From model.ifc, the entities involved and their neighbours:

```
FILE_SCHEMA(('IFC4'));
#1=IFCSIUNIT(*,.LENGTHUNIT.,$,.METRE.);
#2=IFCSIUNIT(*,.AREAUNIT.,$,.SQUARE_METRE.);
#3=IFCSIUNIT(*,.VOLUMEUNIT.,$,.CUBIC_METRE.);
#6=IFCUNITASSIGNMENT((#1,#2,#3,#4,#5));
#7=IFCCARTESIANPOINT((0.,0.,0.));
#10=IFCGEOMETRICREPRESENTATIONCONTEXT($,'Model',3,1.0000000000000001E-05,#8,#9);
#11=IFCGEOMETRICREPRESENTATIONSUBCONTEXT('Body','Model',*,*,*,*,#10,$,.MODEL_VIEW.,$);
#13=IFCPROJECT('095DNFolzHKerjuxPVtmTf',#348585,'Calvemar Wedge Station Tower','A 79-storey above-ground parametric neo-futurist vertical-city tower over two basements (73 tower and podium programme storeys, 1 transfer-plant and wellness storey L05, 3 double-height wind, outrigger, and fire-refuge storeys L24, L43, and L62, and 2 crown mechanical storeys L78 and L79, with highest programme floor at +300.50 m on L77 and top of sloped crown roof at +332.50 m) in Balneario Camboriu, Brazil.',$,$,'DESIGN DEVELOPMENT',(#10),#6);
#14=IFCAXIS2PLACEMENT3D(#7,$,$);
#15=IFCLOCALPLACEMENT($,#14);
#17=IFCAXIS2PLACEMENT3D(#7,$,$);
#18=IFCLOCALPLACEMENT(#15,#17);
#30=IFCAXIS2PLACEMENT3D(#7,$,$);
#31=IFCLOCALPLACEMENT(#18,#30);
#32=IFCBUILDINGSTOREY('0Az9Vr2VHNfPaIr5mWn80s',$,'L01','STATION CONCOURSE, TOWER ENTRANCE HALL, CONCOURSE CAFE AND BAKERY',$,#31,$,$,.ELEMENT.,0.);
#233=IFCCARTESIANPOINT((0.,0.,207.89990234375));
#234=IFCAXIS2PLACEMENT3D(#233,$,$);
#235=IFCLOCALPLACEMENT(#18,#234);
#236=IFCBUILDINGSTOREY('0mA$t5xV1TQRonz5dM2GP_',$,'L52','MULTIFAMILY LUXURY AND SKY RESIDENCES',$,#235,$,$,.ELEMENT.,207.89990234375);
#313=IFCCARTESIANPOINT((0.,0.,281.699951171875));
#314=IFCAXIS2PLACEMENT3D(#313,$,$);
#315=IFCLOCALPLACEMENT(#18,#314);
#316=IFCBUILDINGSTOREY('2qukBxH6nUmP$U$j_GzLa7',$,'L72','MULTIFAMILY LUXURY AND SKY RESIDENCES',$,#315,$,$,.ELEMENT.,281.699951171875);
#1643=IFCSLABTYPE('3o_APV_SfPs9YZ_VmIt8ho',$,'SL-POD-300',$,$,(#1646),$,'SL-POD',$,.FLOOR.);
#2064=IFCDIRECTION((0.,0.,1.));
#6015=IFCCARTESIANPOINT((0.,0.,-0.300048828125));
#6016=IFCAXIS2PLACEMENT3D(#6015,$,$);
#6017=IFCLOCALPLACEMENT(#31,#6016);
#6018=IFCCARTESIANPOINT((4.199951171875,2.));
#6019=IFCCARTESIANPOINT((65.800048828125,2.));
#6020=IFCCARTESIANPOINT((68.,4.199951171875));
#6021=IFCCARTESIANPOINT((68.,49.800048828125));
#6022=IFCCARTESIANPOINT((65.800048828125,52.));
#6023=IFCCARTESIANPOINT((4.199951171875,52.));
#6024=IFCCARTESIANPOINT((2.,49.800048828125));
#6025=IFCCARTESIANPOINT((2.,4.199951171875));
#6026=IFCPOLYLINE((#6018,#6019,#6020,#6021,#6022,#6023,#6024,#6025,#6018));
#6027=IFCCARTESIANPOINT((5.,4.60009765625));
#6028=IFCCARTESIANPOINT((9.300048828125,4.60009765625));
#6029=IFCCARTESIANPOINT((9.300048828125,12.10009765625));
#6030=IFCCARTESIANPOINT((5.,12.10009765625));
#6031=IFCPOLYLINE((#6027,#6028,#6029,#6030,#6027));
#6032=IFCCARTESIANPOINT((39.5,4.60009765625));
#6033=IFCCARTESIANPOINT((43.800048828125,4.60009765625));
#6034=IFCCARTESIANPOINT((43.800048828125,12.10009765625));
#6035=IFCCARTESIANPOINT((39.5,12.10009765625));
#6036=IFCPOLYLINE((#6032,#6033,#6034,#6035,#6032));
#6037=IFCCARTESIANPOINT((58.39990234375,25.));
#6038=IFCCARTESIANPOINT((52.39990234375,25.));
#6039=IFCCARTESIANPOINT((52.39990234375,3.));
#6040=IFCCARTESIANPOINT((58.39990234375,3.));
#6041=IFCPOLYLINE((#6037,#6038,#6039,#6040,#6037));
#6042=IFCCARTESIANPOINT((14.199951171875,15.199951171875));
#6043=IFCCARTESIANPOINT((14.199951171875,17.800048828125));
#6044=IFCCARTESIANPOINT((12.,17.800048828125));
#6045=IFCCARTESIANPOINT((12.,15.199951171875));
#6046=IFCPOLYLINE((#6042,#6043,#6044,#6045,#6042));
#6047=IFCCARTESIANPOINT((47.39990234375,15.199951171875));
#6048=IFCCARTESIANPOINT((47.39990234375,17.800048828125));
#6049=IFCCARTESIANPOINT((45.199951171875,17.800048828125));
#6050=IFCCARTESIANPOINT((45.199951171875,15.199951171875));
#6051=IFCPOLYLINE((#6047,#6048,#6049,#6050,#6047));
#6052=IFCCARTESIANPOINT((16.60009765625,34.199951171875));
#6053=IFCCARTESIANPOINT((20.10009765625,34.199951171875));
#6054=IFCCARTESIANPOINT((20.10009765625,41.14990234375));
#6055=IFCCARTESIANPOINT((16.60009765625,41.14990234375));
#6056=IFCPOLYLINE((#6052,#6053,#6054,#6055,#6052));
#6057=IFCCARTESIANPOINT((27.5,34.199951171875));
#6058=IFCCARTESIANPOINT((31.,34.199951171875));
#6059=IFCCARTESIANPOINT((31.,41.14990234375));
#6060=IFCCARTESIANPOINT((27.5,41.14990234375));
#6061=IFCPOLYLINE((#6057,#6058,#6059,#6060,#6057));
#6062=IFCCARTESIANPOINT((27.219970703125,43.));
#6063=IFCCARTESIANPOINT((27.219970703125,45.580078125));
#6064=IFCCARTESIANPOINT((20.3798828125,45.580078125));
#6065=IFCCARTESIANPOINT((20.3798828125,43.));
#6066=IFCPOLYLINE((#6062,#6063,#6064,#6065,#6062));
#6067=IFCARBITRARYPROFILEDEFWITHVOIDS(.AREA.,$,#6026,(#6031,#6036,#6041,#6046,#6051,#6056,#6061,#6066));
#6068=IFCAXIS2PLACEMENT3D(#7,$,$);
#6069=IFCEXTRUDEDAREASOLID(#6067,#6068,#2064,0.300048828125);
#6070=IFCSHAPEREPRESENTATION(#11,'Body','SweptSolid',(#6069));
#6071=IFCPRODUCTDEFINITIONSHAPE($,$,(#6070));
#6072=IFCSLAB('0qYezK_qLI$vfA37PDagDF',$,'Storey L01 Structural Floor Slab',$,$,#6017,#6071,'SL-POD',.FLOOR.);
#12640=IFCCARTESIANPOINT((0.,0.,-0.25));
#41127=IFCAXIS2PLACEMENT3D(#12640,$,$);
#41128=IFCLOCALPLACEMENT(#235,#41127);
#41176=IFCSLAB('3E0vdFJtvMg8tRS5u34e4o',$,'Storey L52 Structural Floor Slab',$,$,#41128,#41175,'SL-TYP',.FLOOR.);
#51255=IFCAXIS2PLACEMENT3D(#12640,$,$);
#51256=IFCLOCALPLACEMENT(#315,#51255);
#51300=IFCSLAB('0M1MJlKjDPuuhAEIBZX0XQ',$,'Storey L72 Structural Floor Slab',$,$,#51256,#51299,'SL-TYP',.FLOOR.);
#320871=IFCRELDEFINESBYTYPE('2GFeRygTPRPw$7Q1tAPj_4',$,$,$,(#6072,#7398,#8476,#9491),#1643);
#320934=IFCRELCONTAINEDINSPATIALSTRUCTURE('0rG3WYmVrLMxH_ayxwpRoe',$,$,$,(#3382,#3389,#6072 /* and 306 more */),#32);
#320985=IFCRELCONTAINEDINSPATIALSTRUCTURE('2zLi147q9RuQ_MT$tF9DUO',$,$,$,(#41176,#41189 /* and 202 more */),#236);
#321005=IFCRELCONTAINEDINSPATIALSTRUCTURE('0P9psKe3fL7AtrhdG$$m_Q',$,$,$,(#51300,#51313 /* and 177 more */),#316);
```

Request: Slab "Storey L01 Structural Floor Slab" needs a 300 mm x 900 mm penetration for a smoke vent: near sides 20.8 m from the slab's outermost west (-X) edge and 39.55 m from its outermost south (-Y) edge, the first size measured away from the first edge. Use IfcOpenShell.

```python
import numpy as np
import ifcopenshell
import ifcopenshell.api.feature
import ifcopenshell.api.geometry
import ifcopenshell.api.root
import ifcopenshell.geom
import ifcopenshell.util.placement
import ifcopenshell.util.representation
import ifcopenshell.util.shape
import ifcopenshell.util.unit

model = ifcopenshell.open("model.ifc")
unit_scale = ifcopenshell.util.unit.calculate_unit_scale(model)
settings = ifcopenshell.geom.settings()


def volume(element):
    """Net volume in cubic metres, openings subtracted."""
    shape = ifcopenshell.geom.create_shape(settings, element)
    return ifcopenshell.util.shape.get_volume(shape.geometry)


slab = model.by_guid("0qYezK_qLI$vfA37PDagDF")
before = volume(slab)

# Extent in the slab's own axes, in metres. The edges named are its -X and -Y sides.
slab_shape = ifcopenshell.geom.create_shape(settings, slab)
vertices = ifcopenshell.util.shape.get_vertices(slab_shape.geometry)
x_min, y_min, bottom = vertices.min(axis=0)
top = vertices[:, 2].max()

opening = ifcopenshell.api.root.create_entity(model, ifc_class="IfcOpeningElement", name="Smoke vent opening", predefined_type="OPENING")
context = ifcopenshell.util.representation.get_context(model, "Model", "Body", "MODEL_VIEW")
width, depth = 0.3, 0.9
outline = [(0.0, 0.0), (width, 0.0), (width, depth), (0.0, depth), (0.0, 0.0)]
# Overshoot both faces by 50 mm so the cut is clean.
shape = ifcopenshell.api.geometry.add_slab_representation(
    model, context=context, depth=top - bottom + 0.1, polyline=outline
)
ifcopenshell.api.geometry.assign_representation(model, product=opening, representation=shape)

matrix = ifcopenshell.util.placement.get_local_placement(slab.ObjectPlacement)
matrix[:, 3] = matrix @ np.append(np.array([x_min + 20.8, y_min + 39.55, bottom - 0.05]) / unit_scale, 1.0)
ifcopenshell.api.geometry.edit_object_placement(model, product=opening, matrix=matrix, is_si=False)
ifcopenshell.api.feature.add_feature(model, feature=opening, element=slab)

after = volume(slab)

print(f"slab volume {before:.3f} -> {after:.3f} m3")

model.write("model_rev.ifc")
```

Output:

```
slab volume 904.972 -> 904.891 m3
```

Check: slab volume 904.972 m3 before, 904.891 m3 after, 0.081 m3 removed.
